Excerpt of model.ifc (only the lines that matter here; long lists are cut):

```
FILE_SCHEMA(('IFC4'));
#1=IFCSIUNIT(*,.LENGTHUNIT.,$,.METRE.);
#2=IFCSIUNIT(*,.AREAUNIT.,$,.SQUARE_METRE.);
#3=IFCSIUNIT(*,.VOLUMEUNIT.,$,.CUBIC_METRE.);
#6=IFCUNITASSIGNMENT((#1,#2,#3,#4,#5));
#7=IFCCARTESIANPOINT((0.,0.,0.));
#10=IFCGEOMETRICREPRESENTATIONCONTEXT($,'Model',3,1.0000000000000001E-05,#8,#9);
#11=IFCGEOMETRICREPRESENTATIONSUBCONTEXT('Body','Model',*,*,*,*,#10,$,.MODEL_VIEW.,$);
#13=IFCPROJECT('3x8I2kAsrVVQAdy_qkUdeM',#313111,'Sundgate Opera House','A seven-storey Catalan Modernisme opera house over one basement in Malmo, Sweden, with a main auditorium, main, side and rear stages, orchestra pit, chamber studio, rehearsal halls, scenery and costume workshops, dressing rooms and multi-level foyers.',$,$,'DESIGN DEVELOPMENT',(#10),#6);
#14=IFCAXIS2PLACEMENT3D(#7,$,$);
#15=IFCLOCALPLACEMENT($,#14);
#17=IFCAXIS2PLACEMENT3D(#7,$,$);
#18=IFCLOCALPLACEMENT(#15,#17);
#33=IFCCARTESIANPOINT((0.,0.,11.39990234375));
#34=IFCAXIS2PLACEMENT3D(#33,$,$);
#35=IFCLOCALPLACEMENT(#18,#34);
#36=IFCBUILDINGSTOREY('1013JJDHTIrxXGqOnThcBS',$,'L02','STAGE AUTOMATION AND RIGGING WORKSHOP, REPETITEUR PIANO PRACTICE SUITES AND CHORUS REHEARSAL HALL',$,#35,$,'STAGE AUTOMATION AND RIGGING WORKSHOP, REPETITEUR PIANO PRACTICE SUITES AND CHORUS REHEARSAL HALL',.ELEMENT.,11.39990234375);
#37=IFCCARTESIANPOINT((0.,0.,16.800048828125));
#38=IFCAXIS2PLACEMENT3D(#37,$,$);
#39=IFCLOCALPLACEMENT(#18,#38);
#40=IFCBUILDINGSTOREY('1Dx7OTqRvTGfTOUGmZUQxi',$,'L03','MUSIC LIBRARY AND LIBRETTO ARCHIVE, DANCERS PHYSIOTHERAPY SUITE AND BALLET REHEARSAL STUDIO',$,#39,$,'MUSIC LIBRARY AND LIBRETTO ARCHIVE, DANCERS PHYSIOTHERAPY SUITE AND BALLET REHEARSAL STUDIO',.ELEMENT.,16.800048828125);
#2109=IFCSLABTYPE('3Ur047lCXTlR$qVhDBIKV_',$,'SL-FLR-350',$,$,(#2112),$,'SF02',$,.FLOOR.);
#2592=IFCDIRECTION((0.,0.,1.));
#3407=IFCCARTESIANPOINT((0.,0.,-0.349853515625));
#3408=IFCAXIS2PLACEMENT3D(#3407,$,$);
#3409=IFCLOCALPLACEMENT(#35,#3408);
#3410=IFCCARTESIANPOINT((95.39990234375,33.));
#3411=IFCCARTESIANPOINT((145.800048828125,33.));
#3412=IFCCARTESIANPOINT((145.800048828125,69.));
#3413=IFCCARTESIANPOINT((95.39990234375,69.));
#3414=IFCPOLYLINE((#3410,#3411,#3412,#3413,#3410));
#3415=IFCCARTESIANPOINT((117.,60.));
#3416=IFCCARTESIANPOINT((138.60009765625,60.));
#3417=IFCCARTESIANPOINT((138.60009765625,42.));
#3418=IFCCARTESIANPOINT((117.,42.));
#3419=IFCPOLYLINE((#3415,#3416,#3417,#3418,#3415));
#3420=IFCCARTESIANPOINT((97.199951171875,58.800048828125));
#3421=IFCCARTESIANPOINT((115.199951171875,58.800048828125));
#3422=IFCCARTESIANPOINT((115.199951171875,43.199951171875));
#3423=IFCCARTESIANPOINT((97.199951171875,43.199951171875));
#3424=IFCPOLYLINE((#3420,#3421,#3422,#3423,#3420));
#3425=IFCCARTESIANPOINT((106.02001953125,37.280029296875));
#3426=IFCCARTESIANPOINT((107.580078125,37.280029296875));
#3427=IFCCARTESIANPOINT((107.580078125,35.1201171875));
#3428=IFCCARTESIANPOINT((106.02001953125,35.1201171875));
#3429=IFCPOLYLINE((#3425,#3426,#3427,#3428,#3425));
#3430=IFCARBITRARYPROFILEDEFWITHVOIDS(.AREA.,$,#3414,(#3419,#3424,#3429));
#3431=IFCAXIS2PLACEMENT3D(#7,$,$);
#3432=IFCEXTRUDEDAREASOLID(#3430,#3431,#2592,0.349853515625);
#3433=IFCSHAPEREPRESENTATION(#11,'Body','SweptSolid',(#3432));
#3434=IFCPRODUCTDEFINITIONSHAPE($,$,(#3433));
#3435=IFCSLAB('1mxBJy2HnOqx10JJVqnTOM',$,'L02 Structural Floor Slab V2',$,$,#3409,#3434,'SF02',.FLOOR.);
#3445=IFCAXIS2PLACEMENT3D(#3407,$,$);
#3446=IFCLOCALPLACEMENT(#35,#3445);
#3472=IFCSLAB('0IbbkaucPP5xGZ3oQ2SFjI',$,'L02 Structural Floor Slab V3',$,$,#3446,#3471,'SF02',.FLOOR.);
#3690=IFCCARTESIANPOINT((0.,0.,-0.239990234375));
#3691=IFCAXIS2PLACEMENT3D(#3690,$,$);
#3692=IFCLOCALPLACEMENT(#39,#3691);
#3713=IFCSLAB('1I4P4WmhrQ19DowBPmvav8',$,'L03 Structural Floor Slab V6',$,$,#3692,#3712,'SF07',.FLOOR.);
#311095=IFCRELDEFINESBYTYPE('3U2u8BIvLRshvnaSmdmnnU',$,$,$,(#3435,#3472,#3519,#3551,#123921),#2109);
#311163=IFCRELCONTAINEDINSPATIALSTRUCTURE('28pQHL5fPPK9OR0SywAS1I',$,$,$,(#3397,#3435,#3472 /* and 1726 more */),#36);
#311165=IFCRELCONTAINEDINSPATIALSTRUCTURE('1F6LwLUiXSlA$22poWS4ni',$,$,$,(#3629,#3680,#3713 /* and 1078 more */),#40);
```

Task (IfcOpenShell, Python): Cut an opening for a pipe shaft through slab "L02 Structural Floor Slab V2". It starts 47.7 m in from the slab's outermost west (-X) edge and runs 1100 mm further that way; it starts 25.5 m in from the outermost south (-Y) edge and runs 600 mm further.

```python
import numpy as np
import ifcopenshell
import ifcopenshell.api.feature
import ifcopenshell.api.geometry
import ifcopenshell.api.root
import ifcopenshell.geom
import ifcopenshell.util.placement
import ifcopenshell.util.representation
import ifcopenshell.util.shape
import ifcopenshell.util.unit

model = ifcopenshell.open("model.ifc")
unit_scale = ifcopenshell.util.unit.calculate_unit_scale(model)
settings = ifcopenshell.geom.settings()


def volume(element):
    """Net volume in cubic metres, openings subtracted."""
    shape = ifcopenshell.geom.create_shape(settings, element)
    return ifcopenshell.util.shape.get_volume(shape.geometry)


slab = model.by_guid("1mxBJy2HnOqx10JJVqnTOM")
before = volume(slab)

# Extent in the slab's own axes, in metres. The edges named are its -X and -Y sides.
slab_shape = ifcopenshell.geom.create_shape(settings, slab)
vertices = ifcopenshell.util.shape.get_vertices(slab_shape.geometry)
x_min, y_min, bottom = vertices.min(axis=0)
top = vertices[:, 2].max()

opening = ifcopenshell.api.root.create_entity(model, ifc_class="IfcOpeningElement", name="Pipe shaft opening", predefined_type="OPENING")
context = ifcopenshell.util.representation.get_context(model, "Model", "Body", "MODEL_VIEW")
width, depth = 1.1, 0.6
outline = [(0.0, 0.0), (width, 0.0), (width, depth), (0.0, depth), (0.0, 0.0)]
# Overshoot both faces by 50 mm so the cut is clean.
shape = ifcopenshell.api.geometry.add_slab_representation(
    model, context=context, depth=top - bottom + 0.1, polyline=outline
)
ifcopenshell.api.geometry.assign_representation(model, product=opening, representation=shape)

matrix = ifcopenshell.util.placement.get_local_placement(slab.ObjectPlacement)
matrix[:, 3] = matrix @ np.append(np.array([x_min + 47.7, y_min + 25.5, bottom - 0.05]) / unit_scale, 1.0)
ifcopenshell.api.geometry.edit_object_placement(model, product=opening, matrix=matrix, is_si=False)
ifcopenshell.api.feature.add_feature(model, feature=opening, element=slab)

after = volume(slab)

print(f"slab volume {before:.3f} -> {after:.3f} m3")

model.write("model-out.ifc")
```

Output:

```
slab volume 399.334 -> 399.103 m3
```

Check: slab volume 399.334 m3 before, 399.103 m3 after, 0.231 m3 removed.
